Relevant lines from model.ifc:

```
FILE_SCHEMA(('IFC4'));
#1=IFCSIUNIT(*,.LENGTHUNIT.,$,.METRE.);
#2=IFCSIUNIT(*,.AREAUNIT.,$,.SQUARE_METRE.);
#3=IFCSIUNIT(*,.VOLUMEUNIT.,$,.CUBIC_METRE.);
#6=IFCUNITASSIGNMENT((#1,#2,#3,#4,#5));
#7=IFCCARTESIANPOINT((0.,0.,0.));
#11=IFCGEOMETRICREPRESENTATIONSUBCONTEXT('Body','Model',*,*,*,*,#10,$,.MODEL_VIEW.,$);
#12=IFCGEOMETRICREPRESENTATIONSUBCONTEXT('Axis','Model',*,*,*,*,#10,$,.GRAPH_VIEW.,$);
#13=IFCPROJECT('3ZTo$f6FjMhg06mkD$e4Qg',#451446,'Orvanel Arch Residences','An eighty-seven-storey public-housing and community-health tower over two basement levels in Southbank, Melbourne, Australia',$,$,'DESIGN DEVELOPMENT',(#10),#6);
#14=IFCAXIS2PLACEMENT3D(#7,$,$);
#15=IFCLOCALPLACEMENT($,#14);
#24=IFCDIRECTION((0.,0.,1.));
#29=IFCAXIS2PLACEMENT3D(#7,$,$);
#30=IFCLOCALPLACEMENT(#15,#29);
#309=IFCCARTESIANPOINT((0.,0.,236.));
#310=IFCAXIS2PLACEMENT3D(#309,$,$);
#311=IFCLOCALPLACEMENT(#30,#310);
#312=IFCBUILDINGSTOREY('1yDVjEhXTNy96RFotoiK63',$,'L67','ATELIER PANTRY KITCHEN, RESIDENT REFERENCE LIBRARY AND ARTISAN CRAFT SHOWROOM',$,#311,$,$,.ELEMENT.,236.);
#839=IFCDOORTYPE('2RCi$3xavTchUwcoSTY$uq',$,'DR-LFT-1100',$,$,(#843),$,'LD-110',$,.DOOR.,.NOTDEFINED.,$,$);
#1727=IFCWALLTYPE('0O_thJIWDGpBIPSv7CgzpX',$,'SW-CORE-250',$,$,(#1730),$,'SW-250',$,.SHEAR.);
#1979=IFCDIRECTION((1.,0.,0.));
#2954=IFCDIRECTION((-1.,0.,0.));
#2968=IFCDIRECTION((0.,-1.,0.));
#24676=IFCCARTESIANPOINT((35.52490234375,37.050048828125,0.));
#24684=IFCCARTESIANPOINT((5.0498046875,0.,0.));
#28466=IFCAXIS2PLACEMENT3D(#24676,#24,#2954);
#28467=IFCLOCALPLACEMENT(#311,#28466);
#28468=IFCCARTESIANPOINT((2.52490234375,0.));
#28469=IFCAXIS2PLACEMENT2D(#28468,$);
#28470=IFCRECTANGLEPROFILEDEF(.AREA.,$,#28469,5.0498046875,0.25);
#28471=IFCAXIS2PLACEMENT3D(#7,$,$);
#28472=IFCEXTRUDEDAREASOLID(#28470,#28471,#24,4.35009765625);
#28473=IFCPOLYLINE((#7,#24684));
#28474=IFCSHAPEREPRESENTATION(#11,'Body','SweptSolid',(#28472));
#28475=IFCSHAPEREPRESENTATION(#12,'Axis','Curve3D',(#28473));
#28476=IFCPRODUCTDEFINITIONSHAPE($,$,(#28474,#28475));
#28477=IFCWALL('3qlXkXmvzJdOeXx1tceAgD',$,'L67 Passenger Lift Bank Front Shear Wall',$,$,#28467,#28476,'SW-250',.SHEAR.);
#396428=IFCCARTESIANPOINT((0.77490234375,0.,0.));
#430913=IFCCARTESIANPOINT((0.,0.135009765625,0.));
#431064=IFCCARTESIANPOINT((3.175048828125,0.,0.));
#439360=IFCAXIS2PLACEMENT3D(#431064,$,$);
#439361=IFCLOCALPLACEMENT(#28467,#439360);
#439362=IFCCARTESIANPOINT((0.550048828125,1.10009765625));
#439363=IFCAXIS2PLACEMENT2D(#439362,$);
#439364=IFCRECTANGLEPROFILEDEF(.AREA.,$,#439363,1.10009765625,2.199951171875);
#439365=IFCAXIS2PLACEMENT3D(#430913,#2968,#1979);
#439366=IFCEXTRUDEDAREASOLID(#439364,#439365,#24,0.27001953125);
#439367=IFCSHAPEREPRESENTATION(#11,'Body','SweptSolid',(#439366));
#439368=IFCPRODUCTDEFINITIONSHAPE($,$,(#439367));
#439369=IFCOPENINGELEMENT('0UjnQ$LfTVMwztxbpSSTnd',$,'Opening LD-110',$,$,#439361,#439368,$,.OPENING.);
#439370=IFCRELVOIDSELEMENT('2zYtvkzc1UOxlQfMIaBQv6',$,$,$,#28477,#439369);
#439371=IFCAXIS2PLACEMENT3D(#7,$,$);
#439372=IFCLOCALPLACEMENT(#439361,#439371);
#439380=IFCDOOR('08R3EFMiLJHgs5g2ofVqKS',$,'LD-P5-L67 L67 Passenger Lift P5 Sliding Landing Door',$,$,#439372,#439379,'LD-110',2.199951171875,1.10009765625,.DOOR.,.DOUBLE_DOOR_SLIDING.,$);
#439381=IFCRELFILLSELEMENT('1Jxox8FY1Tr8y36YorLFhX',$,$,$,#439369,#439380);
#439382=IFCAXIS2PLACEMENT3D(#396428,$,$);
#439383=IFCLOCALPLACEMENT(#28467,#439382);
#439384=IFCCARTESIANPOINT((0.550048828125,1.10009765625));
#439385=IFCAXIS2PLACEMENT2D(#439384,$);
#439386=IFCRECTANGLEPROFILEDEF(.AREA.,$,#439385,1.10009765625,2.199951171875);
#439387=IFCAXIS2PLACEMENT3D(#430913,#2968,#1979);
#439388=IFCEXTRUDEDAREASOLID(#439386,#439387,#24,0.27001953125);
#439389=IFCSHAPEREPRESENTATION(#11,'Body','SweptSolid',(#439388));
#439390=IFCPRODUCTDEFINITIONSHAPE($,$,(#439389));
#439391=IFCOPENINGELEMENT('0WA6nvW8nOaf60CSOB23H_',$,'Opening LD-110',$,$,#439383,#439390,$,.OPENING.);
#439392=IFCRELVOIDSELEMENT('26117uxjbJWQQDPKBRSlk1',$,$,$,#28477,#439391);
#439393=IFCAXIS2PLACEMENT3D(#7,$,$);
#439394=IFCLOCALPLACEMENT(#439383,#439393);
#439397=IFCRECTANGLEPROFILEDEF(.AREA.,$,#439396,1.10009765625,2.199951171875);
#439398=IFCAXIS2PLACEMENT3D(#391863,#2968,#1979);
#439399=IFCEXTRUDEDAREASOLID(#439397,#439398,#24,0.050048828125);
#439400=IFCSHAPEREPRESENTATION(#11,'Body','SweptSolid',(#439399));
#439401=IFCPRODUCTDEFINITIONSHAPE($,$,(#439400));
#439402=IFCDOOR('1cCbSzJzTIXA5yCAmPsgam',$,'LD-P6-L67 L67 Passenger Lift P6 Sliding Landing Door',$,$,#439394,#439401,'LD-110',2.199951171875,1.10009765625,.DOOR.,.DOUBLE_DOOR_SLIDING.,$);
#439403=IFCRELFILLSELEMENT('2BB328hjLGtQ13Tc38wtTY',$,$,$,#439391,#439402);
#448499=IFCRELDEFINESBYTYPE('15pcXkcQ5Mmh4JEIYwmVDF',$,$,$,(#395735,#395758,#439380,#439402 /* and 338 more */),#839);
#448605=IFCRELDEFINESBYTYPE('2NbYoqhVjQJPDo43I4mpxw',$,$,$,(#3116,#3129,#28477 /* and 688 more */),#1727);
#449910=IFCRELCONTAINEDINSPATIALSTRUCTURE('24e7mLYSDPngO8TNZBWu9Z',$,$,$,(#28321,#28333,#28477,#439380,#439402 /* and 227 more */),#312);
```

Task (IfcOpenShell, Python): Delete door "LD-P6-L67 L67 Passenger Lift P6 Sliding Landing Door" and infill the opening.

```python
import ifcopenshell
import ifcopenshell.api.feature
import ifcopenshell.api.root
import ifcopenshell.geom
import ifcopenshell.util.shape

model = ifcopenshell.open("model.ifc")
settings = ifcopenshell.geom.settings()


def volume(element):
    """Net volume in cubic metres, openings subtracted."""
    shape = ifcopenshell.geom.create_shape(settings, element)
    return ifcopenshell.util.shape.get_volume(shape.geometry)


door = model.by_guid("1cCbSzJzTIXA5yCAmPsgam")
opening = door.FillsVoids[0].RelatingOpeningElement
wall = opening.VoidsElements[0].RelatingBuildingElement
before = volume(wall)

ifcopenshell.api.root.remove_product(model, product=door)
ifcopenshell.api.feature.remove_feature(model, feature=opening)

after = volume(wall)

print(f"wall volume {before:.3f} -> {after:.3f} m3")

model.write("model_v2.ifc")
```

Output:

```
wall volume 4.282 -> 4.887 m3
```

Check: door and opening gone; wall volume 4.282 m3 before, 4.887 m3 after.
